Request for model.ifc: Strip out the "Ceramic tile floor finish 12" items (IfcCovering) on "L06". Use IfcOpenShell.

First a look at what the model holds.

```python
import ifcopenshell
import ifcopenshell.util.element

model = ifcopenshell.open("model.ifc")
print(model.schema)
storey = next(s for s in model.by_type("IfcBuildingStorey") if s.Name == "L06")
coverings = [e for e in ifcopenshell.util.element.get_decomposition(storey) if e.is_a("IfcCovering")]
seen = {}
for e in coverings:
    element_type = ifcopenshell.util.element.get_type(e)
    name = element_type.Name if element_type not in (None, e) else None
    seen[name] = seen.get(name, 0) + 1
for name, count in sorted(seen.items(), key=str):
    print(count, "x", name)
```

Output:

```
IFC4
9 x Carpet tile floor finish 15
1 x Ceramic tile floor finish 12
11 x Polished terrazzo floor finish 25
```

```python
import ifcopenshell
import ifcopenshell.api.root
import ifcopenshell.util.element

model = ifcopenshell.open("model.ifc")

storey = next(s for s in model.by_type("IfcBuildingStorey") if s.Name == "L06")
coverings = [e for e in ifcopenshell.util.element.get_decomposition(storey) if e.is_a("IfcCovering")]
targets = [e for e in coverings if (t := ifcopenshell.util.element.get_type(e)) not in (None, e) and t.Name == "Ceramic tile floor finish 12"]

for e in targets:
    ifcopenshell.api.root.remove_product(model, product=e)
print(len(targets), "removed")

model.write("model_rev.ifc")
```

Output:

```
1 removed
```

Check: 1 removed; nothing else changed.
